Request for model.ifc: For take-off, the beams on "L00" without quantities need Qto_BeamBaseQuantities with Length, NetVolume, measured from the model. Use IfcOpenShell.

First a look at what the model holds.

```python
import ifcopenshell
import ifcopenshell.util.element
import ifcopenshell.util.unit

model = ifcopenshell.open("model.ifc")
print(model.schema)
for unit_type in ("LENGTHUNIT", "AREAUNIT", "VOLUMEUNIT"):
    print(unit_type, ifcopenshell.util.unit.calculate_unit_scale(model, unit_type))
storey = next(s for s in model.by_type("IfcBuildingStorey") if s.Name == "L00")
beams = [e for e in ifcopenshell.util.element.get_decomposition(storey) if e.is_a("IfcBeam")]
for e in sorted(beams, key=lambda e: e.id()):
    print(e.id(), e.is_a(), e.Name, list(ifcopenshell.util.element.get_psets(e, qtos_only=True)), sep=" | ")
```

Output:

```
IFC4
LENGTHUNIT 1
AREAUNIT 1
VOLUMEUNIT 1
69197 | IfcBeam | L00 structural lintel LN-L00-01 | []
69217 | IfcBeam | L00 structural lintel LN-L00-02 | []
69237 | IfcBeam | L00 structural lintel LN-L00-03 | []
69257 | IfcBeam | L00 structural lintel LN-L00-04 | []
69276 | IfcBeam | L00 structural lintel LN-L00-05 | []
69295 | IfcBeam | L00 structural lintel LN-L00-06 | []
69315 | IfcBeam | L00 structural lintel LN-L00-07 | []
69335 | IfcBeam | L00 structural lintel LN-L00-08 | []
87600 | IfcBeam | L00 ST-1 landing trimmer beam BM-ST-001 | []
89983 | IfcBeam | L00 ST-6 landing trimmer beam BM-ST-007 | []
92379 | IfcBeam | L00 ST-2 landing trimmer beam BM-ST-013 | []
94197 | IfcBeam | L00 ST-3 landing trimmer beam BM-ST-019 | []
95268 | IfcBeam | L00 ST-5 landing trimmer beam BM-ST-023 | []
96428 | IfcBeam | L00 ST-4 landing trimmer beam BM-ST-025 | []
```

```python
import ifcopenshell
import ifcopenshell.api.pset
import ifcopenshell.geom
import ifcopenshell.util.element
import ifcopenshell.util.shape
import ifcopenshell.util.unit

model = ifcopenshell.open("model.ifc")
unit_scale = ifcopenshell.util.unit.calculate_unit_scale(model)
volume_scale = ifcopenshell.util.unit.calculate_unit_scale(model, "VOLUMEUNIT")
settings = ifcopenshell.geom.settings()

storey = next(s for s in model.by_type("IfcBuildingStorey") if s.Name == "L00")
beams = [e for e in ifcopenshell.util.element.get_decomposition(storey) if e.is_a("IfcBeam")]

for e in sorted(beams, key=lambda e: e.id()):
    if ifcopenshell.util.element.get_psets(e, qtos_only=True, should_inherit=False):
        continue
    # Geometry comes back in metres, in the element's own axes.
    shape = ifcopenshell.geom.create_shape(settings, e)
    values = {
        "Length": ifcopenshell.util.shape.get_max_xyz(shape.geometry) / unit_scale,
        "NetVolume": ifcopenshell.util.shape.get_volume(shape.geometry) / volume_scale,
    }
    qto = ifcopenshell.api.pset.add_qto(model, product=e, name="Qto_BeamBaseQuantities")
    ifcopenshell.api.pset.edit_qto(model, qto=qto, properties=values)
    print(e.id(), {k: round(v, 3) for k, v in values.items()})

model.write("model_v2.ifc")
```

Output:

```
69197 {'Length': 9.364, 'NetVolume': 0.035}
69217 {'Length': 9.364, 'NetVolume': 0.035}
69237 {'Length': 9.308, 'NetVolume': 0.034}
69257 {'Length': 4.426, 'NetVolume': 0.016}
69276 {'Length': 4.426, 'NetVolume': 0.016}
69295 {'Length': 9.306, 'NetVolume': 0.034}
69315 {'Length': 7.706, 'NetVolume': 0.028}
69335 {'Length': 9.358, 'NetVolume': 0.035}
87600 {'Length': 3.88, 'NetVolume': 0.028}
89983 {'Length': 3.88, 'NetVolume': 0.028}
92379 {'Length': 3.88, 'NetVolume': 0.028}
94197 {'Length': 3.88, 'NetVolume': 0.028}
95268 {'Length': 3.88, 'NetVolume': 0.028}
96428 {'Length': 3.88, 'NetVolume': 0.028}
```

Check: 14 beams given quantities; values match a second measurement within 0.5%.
